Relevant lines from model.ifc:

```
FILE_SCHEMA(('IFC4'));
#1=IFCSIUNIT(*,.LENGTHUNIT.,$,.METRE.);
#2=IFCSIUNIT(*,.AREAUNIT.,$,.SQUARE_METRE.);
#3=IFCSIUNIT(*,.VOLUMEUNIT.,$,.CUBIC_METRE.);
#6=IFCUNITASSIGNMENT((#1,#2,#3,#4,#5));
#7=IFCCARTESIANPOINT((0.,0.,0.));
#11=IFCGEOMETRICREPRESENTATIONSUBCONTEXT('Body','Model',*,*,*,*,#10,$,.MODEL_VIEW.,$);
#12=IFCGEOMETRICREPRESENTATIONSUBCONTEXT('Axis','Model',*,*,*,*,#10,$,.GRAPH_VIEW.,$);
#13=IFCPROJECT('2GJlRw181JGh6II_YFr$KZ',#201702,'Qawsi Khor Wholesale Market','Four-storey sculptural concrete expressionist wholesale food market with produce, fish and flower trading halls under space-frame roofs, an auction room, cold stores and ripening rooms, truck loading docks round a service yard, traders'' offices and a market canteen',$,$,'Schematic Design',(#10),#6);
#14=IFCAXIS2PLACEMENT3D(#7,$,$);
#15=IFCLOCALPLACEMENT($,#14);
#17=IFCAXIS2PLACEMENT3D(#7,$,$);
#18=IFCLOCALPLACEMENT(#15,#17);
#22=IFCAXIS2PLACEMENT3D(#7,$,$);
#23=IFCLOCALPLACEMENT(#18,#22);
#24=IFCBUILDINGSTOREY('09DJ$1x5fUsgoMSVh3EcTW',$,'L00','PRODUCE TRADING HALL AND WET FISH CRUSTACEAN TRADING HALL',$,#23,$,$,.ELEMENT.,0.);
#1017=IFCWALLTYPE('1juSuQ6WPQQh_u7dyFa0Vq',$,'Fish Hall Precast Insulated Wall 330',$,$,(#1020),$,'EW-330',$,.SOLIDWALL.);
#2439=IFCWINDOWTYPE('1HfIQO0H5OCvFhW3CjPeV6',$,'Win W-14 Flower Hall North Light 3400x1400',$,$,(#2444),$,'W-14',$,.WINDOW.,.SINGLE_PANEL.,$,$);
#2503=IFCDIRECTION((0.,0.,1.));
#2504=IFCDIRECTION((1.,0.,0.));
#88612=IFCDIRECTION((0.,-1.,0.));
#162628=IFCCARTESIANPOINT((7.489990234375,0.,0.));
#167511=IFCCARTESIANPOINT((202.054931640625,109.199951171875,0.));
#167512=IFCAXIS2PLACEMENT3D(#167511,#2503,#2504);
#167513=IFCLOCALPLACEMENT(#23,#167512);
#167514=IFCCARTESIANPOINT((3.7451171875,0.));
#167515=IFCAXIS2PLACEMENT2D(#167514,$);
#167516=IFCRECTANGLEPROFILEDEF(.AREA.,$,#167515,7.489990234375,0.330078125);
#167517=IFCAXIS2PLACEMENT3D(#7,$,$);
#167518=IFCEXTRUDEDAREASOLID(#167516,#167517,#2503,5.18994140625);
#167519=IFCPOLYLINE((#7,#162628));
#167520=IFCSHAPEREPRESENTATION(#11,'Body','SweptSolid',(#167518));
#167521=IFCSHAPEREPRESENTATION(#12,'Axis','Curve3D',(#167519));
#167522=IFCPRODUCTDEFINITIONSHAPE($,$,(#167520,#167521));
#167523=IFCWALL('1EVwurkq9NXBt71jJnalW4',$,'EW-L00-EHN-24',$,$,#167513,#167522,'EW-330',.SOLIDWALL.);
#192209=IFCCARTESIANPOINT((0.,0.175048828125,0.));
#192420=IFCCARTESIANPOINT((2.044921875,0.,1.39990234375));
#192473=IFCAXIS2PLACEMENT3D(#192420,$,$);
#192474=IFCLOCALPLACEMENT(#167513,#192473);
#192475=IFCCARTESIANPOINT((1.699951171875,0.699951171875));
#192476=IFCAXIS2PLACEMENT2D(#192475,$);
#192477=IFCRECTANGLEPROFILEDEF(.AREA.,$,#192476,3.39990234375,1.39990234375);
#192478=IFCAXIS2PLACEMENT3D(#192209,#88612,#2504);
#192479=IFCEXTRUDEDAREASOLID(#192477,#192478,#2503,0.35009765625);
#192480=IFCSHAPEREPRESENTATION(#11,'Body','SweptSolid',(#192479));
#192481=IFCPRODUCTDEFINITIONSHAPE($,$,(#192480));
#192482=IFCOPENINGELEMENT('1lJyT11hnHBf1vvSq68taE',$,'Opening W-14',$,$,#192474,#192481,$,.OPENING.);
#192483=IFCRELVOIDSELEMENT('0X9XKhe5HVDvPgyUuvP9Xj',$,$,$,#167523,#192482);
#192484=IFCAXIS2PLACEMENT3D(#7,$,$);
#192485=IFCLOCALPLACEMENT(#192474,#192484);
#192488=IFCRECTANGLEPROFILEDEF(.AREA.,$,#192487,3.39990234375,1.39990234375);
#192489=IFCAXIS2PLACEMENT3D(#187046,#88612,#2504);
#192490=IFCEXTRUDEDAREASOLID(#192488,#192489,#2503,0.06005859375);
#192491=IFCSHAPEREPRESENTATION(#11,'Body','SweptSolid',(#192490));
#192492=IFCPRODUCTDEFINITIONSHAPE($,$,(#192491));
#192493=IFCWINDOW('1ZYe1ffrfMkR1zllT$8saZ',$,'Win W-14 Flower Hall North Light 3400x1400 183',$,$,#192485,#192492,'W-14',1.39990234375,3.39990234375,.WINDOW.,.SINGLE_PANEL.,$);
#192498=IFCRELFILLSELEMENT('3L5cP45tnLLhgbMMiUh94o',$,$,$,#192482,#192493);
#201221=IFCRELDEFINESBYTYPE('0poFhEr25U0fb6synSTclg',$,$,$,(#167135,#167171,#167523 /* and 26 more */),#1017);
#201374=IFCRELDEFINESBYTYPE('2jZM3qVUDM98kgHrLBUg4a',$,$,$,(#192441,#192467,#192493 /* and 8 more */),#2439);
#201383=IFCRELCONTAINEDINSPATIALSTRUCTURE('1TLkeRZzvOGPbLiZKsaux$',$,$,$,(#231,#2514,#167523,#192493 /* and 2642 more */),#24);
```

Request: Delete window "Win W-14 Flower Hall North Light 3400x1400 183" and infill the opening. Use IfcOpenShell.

```python
import ifcopenshell
import ifcopenshell.api.feature
import ifcopenshell.api.root
import ifcopenshell.geom
import ifcopenshell.util.shape

model = ifcopenshell.open("model.ifc")
settings = ifcopenshell.geom.settings()


def volume(element):
    """Net volume in cubic metres, openings subtracted."""
    shape = ifcopenshell.geom.create_shape(settings, element)
    return ifcopenshell.util.shape.get_volume(shape.geometry)


window = model.by_guid("1ZYe1ffrfMkR1zllT$8saZ")
opening = window.FillsVoids[0].RelatingOpeningElement
wall = opening.VoidsElements[0].RelatingBuildingElement
before = volume(wall)

ifcopenshell.api.root.remove_product(model, product=window)
ifcopenshell.api.feature.remove_feature(model, feature=opening)

after = volume(wall)

print(f"wall volume {before:.3f} -> {after:.3f} m3")

model.write("model_rev.ifc")
```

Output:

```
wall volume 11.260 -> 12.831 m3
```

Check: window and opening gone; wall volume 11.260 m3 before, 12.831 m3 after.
